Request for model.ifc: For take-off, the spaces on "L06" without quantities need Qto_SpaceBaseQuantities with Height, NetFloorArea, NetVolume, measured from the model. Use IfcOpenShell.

First a look at what the model holds.

```python
import ifcopenshell
import ifcopenshell.util.element
import ifcopenshell.util.unit

model = ifcopenshell.open("model.ifc")
print(model.schema)
for unit_type in ("LENGTHUNIT", "AREAUNIT", "VOLUMEUNIT"):
    print(unit_type, ifcopenshell.util.unit.calculate_unit_scale(model, unit_type))
storey = next(s for s in model.by_type("IfcBuildingStorey") if s.Name == "L06")
spaces = [e for e in ifcopenshell.util.element.get_decomposition(storey) if e.is_a("IfcSpace")]
for e in sorted(spaces, key=lambda e: e.id()):
    print(e.id(), e.is_a(), e.Name, list(ifcopenshell.util.element.get_psets(e, qtos_only=True)), sep=" | ")
```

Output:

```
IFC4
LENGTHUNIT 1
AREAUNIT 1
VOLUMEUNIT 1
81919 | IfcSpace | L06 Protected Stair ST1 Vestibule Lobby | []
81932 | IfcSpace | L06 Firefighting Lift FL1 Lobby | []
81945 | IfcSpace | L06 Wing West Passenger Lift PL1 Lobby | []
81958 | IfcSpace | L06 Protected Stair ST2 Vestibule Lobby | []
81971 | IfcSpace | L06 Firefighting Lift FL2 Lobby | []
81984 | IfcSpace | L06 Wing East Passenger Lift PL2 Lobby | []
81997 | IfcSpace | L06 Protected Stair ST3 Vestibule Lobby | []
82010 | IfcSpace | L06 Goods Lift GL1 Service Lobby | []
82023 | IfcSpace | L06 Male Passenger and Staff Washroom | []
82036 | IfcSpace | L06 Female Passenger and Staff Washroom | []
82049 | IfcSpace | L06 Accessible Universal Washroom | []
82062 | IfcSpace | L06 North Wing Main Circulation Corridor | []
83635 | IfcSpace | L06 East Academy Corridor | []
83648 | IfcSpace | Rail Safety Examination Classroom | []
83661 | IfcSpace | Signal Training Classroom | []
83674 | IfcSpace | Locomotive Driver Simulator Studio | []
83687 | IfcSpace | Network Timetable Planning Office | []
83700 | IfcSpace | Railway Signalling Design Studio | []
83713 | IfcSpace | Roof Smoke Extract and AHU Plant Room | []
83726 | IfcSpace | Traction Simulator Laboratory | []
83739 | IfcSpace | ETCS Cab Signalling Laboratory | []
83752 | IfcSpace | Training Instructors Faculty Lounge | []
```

```python
import ifcopenshell
import ifcopenshell.api.pset
import ifcopenshell.geom
import ifcopenshell.util.element
import ifcopenshell.util.shape
import ifcopenshell.util.unit

model = ifcopenshell.open("model.ifc")
unit_scale = ifcopenshell.util.unit.calculate_unit_scale(model)
area_scale = ifcopenshell.util.unit.calculate_unit_scale(model, "AREAUNIT")
volume_scale = ifcopenshell.util.unit.calculate_unit_scale(model, "VOLUMEUNIT")
settings = ifcopenshell.geom.settings()

storey = next(s for s in model.by_type("IfcBuildingStorey") if s.Name == "L06")
spaces = [e for e in ifcopenshell.util.element.get_decomposition(storey) if e.is_a("IfcSpace")]

for e in sorted(spaces, key=lambda e: e.id()):
    if ifcopenshell.util.element.get_psets(e, qtos_only=True, should_inherit=False):
        continue
    # Geometry comes back in metres, in the element's own axes.
    shape = ifcopenshell.geom.create_shape(settings, e)
    values = {
        "Height": ifcopenshell.util.shape.get_z(shape.geometry) / unit_scale,
        "NetFloorArea": ifcopenshell.util.shape.get_footprint_area(shape.geometry) / area_scale,
        "NetVolume": ifcopenshell.util.shape.get_volume(shape.geometry) / volume_scale,
    }
    qto = ifcopenshell.api.pset.add_qto(model, product=e, name="Qto_SpaceBaseQuantities")
    ifcopenshell.api.pset.edit_qto(model, qto=qto, properties=values)
    print(e.id(), {k: round(v, 3) for k, v in values.items()})

model.write("model-out.ifc")
```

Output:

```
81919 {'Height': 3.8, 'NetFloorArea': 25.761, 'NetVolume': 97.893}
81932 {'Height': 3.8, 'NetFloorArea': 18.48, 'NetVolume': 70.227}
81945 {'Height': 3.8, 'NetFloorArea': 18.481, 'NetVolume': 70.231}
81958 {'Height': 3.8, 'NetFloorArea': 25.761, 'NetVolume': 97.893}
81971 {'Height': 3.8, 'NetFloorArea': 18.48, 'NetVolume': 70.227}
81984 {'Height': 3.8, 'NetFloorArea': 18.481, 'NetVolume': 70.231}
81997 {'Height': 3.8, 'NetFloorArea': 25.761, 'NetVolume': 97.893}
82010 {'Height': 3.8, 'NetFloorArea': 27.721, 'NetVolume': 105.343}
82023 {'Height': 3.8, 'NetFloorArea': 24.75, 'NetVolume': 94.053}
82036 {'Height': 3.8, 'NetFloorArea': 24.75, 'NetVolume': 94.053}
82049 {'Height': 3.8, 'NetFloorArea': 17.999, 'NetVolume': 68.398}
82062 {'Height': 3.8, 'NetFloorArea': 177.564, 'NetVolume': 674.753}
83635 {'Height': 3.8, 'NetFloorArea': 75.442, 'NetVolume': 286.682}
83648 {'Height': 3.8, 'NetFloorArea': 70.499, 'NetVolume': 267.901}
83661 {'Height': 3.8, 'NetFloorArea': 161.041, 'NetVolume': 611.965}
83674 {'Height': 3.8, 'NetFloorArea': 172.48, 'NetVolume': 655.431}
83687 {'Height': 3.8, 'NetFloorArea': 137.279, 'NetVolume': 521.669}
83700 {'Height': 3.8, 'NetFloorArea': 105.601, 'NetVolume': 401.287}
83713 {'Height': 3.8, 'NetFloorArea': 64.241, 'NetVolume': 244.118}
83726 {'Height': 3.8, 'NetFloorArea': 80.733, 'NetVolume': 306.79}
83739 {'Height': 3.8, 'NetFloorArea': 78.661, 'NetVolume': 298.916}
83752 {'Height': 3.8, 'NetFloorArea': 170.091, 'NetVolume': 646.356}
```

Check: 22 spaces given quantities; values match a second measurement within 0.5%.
